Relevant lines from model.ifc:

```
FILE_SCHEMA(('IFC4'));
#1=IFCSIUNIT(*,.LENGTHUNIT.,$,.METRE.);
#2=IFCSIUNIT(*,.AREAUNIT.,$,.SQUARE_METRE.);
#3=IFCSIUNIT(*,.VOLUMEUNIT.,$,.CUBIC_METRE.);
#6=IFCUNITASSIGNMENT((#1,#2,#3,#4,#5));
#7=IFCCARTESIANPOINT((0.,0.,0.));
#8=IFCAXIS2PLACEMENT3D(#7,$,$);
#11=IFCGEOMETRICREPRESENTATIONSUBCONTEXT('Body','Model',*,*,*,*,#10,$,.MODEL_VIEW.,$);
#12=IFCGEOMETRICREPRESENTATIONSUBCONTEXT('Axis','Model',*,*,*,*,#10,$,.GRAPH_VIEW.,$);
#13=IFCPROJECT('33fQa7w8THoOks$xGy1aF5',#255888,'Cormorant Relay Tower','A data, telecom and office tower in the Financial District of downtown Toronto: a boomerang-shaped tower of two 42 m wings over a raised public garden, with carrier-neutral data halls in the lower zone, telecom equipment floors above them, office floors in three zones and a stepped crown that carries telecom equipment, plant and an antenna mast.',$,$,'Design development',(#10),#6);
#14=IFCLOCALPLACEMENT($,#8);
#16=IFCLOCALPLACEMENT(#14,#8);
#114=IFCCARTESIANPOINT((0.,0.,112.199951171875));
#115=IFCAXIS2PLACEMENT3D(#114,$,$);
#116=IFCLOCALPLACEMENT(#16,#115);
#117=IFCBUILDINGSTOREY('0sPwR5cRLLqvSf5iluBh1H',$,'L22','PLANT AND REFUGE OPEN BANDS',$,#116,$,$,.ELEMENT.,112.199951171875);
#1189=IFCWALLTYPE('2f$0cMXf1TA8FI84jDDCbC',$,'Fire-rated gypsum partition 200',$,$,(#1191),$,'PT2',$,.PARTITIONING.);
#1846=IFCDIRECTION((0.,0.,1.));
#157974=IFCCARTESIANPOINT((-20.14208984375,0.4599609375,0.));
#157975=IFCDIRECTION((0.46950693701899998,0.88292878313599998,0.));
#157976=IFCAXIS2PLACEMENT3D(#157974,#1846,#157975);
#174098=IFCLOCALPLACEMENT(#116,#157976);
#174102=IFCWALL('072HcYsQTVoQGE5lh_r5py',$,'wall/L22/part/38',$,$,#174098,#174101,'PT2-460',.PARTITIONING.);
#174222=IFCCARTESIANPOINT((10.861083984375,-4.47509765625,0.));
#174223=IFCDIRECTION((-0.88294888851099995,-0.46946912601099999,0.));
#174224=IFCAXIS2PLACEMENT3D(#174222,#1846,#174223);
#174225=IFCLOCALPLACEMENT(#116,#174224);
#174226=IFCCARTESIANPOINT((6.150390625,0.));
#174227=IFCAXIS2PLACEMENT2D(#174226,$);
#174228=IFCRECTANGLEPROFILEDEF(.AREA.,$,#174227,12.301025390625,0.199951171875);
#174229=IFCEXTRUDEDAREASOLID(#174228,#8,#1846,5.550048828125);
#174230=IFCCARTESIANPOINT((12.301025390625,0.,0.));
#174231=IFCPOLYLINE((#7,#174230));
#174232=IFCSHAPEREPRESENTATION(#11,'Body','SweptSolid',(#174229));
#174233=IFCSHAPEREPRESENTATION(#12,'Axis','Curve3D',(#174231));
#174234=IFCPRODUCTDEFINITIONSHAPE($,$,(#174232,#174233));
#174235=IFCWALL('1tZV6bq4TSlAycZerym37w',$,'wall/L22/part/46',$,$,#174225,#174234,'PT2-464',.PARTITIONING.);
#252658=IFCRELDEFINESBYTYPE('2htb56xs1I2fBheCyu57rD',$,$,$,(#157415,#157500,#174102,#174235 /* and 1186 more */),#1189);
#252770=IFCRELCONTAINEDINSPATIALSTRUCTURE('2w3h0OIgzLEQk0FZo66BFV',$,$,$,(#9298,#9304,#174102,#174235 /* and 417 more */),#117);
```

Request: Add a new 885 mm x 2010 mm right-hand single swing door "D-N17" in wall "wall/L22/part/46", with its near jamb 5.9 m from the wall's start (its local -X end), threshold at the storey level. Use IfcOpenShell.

```python
import numpy as np
import ifcopenshell
import ifcopenshell.api.feature
import ifcopenshell.api.geometry
import ifcopenshell.api.root
import ifcopenshell.api.spatial
import ifcopenshell.geom
import ifcopenshell.util.element
import ifcopenshell.util.placement
import ifcopenshell.util.representation
import ifcopenshell.util.shape
import ifcopenshell.util.unit

model = ifcopenshell.open("model.ifc")
unit_scale = ifcopenshell.util.unit.calculate_unit_scale(model)
settings = ifcopenshell.geom.settings()


def volume(element):
    """Net volume in cubic metres, openings subtracted."""
    shape = ifcopenshell.geom.create_shape(settings, element)
    return ifcopenshell.util.shape.get_volume(shape.geometry)


wall = model.by_id(174235)
storey = ifcopenshell.util.element.get_container(wall, ifc_class="IfcBuildingStorey")
context = ifcopenshell.util.representation.get_context(model, "Model", "Body", "MODEL_VIEW")
before = volume(wall)

width, height, from_end, sill = 0.885, 2.01, 5.9, 0.0  # metres

# The wall runs along its own X axis, and the end named is its -X end.
wall_shape = ifcopenshell.geom.create_shape(settings, wall)
x, y, z = ifcopenshell.util.shape.get_vertices(wall_shape.geometry).T
start = x.min() + from_end
face, thickness = float(y.min()), float(y.max() - y.min())
wall_matrix = ifcopenshell.util.placement.get_local_placement(wall.ObjectPlacement)
level = ifcopenshell.util.placement.get_local_placement(storey.ObjectPlacement)[2, 3]


def in_wall(x, y):
    """Placement at x, y metres in the wall's axes, at sill height."""
    matrix = wall_matrix.copy()
    matrix[:, 3] = wall_matrix @ np.array([x / unit_scale, y / unit_scale, 0.0, 1.0])
    matrix[2, 3] = level + sill / unit_scale
    return matrix


# Opening: a box that overshoots both wall faces by 50 mm.
opening = ifcopenshell.api.root.create_entity(model, ifc_class="IfcOpeningElement", predefined_type="OPENING")
box = ifcopenshell.api.geometry.add_wall_representation(
    model, context=context, length=width, height=height, thickness=thickness + 0.1
)
ifcopenshell.api.geometry.assign_representation(model, product=opening, representation=box)
ifcopenshell.api.geometry.edit_object_placement(model, product=opening, matrix=in_wall(start, face - 0.05), is_si=False)
ifcopenshell.api.feature.add_feature(model, feature=opening, element=wall)

door = ifcopenshell.api.root.create_entity(model, ifc_class="IfcDoor", name="D-N17", predefined_type="DOOR")
door.OverallWidth, door.OverallHeight = width / unit_scale, height / unit_scale
door.OperationType = "SINGLE_SWING_RIGHT"
body = ifcopenshell.api.geometry.add_door_representation(
    model,
    context=context,
    overall_width=door.OverallWidth,
    overall_height=door.OverallHeight,
    operation_type="SINGLE_SWING_RIGHT",
    lining_properties={"LiningDepth": thickness / unit_scale, "ThresholdDepth": thickness / unit_scale},
)
ifcopenshell.api.geometry.assign_representation(model, product=door, representation=body)
ifcopenshell.api.spatial.assign_container(model, products=[door], relating_structure=storey)
ifcopenshell.api.feature.add_filling(model, opening=opening, element=door)

# The lining spans the wall, so the door starts at the wall face.
ifcopenshell.api.geometry.edit_object_placement(model, product=door, matrix=in_wall(start, face), is_si=False)

after = volume(wall)

print(f"wall volume {before:.3f} -> {after:.3f} m3")

model.write("model-out.ifc")
```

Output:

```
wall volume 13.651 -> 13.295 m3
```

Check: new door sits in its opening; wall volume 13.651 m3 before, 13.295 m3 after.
